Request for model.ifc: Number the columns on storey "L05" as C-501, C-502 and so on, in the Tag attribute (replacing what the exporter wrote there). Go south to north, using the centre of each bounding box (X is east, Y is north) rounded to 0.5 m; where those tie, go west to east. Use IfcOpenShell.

First a look at what the model holds.

```python
import ifcopenshell
import ifcopenshell.util.element
import ifcopenshell.util.placement

model = ifcopenshell.open("model.ifc")
print(model.schema)
storey = next(s for s in model.by_type("IfcBuildingStorey") if s.Name == "L05")
columns = [e for e in ifcopenshell.util.element.get_decomposition(storey) if e.is_a("IfcColumn")]
for e in sorted(columns, key=lambda e: e.id()):
    origin = ifcopenshell.util.placement.get_local_placement(e.ObjectPlacement)[:3, 3]
    print(e.id(), e.Tag, e.Name, origin.round(2) + 0.0, sep=" | ")
```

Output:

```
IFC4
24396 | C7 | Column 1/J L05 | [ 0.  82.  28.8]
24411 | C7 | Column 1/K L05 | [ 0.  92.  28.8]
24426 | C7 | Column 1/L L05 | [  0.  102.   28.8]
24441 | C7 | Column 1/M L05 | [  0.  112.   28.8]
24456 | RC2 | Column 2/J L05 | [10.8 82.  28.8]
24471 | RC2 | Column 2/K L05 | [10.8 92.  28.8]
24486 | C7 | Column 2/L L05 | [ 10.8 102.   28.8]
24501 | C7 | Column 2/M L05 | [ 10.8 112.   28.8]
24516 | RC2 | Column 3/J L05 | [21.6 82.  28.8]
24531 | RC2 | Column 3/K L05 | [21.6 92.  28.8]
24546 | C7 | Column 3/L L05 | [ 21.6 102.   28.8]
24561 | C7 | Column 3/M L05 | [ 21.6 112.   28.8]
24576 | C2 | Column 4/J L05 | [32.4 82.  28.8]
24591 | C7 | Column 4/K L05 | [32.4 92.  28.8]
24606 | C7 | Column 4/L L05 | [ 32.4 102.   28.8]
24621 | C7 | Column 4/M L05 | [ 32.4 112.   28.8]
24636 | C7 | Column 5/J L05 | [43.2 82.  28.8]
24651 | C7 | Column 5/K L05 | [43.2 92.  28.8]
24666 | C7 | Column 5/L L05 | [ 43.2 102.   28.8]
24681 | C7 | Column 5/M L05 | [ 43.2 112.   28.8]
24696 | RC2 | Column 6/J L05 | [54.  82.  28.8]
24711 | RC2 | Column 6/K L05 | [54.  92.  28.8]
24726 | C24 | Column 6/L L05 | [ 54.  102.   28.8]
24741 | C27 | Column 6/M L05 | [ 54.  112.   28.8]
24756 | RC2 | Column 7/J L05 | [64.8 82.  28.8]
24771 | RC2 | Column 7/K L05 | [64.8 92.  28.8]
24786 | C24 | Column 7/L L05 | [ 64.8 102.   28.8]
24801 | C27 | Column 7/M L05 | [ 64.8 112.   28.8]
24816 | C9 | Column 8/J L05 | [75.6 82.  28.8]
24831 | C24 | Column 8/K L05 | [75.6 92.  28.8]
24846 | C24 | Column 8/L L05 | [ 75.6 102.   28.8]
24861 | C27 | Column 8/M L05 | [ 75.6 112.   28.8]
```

```python
import ifcopenshell
import ifcopenshell.geom
import ifcopenshell.util.element
import ifcopenshell.util.shape

model = ifcopenshell.open("model.ifc")
settings = ifcopenshell.geom.settings()
settings.set("use-world-coords", True)


def centre(element):
    shape = ifcopenshell.geom.create_shape(settings, element)
    return ifcopenshell.util.shape.get_bbox_centroid(shape.geometry)


storey = next(s for s in model.by_type("IfcBuildingStorey") if s.Name == "L05")
columns = [e for e in ifcopenshell.util.element.get_decomposition(storey) if e.is_a("IfcColumn")]

# Insertion points can sit at a corner or the storey origin, so sort by the geometry (in metres).
centres = {e: centre(e) for e in columns}
columns.sort(key=lambda e: (round(centres[e][1] / 0.5), centres[e][0]))

for i, e in enumerate(columns, start=1):
    number = f"C-5{i:02d}"
    e.Tag = number
    print(e.id(), number)

model.write("model-out.ifc")
```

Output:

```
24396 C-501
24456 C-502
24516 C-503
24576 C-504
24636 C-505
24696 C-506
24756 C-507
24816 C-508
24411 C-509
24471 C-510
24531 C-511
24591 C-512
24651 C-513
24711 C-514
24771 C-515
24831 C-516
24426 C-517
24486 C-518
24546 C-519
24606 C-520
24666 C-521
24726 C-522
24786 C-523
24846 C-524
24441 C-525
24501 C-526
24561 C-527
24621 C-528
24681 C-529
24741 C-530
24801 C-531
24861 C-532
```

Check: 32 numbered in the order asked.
